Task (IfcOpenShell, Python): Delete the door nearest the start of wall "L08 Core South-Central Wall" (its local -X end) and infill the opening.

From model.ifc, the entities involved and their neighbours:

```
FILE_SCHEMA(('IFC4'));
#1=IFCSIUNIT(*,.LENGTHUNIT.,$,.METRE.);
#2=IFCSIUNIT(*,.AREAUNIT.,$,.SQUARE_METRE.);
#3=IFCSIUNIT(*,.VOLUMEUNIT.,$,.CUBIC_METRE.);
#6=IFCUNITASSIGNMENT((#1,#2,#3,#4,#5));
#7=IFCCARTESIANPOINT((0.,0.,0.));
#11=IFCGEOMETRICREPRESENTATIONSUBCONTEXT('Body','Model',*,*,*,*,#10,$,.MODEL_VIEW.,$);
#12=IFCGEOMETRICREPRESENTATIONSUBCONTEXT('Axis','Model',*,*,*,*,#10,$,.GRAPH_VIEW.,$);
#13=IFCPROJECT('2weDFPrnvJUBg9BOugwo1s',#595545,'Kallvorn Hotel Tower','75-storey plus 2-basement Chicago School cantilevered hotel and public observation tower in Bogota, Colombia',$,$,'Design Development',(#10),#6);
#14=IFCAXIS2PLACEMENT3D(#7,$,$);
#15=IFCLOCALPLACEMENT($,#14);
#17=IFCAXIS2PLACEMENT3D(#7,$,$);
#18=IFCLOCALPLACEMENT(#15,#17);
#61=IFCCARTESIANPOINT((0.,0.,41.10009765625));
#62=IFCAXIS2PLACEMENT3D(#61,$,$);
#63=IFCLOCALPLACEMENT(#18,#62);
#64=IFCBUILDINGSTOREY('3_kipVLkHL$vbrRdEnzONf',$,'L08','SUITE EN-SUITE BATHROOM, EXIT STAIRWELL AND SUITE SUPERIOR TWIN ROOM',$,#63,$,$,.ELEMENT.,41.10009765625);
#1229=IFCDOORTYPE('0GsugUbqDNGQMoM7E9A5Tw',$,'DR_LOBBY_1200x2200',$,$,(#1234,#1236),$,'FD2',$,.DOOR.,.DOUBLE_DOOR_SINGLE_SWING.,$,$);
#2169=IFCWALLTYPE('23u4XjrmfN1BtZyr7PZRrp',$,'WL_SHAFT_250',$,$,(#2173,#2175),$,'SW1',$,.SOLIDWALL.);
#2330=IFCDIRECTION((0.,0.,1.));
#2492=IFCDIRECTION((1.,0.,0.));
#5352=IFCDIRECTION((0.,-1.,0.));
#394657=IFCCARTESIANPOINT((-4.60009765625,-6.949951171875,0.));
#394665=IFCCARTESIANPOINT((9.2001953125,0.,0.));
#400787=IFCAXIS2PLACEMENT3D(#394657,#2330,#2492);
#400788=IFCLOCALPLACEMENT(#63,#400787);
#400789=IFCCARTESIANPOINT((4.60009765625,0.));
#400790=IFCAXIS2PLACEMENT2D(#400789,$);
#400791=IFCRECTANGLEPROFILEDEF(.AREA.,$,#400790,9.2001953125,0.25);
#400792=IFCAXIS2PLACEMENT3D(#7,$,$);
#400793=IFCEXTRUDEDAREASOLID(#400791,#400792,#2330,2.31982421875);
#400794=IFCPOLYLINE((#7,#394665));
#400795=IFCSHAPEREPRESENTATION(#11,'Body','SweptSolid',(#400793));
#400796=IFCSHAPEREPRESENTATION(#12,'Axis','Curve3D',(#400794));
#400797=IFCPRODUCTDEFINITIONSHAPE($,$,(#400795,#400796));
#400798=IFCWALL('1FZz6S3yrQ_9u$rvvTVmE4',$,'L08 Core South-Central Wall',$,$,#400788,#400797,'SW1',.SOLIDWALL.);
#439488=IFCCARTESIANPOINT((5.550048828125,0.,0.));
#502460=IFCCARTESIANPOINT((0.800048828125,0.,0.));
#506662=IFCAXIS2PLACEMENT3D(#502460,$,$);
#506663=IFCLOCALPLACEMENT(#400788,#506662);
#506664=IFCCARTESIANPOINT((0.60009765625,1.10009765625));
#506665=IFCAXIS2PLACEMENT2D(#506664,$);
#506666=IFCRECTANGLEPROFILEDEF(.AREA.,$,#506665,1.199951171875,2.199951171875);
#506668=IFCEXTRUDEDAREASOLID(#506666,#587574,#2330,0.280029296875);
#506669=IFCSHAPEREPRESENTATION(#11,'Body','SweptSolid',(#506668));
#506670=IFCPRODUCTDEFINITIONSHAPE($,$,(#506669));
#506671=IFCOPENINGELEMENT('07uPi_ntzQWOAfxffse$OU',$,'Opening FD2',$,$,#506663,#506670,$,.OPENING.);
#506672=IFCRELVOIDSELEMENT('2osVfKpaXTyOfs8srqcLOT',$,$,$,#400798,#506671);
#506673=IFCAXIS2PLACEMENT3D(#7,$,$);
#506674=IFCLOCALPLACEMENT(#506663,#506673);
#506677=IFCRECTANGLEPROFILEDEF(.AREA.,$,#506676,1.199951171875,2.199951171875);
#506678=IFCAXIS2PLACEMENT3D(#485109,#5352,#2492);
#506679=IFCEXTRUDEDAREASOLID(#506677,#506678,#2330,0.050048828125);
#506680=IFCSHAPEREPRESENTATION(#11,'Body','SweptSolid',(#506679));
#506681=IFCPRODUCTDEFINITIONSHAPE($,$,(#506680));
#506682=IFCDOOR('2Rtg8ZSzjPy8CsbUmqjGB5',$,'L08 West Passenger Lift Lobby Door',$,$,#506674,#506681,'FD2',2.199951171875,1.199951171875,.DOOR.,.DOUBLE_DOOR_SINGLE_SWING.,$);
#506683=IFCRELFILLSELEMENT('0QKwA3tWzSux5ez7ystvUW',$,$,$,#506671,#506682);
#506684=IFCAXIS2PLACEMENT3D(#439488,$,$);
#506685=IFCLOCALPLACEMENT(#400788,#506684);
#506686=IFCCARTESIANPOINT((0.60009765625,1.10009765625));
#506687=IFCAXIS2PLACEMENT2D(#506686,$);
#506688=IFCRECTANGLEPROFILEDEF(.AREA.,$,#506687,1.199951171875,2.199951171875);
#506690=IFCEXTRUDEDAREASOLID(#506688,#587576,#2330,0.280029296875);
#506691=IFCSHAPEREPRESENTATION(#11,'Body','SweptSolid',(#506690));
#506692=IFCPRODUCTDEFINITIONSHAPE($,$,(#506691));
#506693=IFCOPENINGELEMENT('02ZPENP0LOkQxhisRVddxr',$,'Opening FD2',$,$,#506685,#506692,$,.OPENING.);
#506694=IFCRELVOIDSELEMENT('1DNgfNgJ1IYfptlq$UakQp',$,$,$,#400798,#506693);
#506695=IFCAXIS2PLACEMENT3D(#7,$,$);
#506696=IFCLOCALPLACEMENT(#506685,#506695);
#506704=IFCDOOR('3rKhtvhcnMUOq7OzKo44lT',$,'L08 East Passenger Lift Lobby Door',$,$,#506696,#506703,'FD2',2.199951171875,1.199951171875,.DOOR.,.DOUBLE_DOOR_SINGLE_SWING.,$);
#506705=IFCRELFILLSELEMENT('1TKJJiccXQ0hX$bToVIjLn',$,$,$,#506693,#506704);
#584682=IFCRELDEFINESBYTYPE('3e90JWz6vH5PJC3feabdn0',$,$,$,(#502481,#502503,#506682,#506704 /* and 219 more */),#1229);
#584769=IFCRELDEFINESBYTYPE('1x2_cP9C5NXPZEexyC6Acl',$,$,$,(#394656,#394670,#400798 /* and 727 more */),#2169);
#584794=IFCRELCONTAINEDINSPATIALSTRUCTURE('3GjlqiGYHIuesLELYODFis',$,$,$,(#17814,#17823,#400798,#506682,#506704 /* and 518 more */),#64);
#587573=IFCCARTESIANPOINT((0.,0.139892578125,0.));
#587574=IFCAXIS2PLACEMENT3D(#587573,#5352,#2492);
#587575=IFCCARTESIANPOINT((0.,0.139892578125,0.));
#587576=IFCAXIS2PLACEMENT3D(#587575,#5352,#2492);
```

```python
import ifcopenshell
import ifcopenshell.api.feature
import ifcopenshell.api.root
import ifcopenshell.geom
import ifcopenshell.util.shape

model = ifcopenshell.open("model.ifc")
settings = ifcopenshell.geom.settings()


def volume(element):
    """Net volume in cubic metres, openings subtracted."""
    shape = ifcopenshell.geom.create_shape(settings, element)
    return ifcopenshell.util.shape.get_volume(shape.geometry)


door = model.by_guid("2Rtg8ZSzjPy8CsbUmqjGB5")
opening = door.FillsVoids[0].RelatingOpeningElement
wall = opening.VoidsElements[0].RelatingBuildingElement
before = volume(wall)

ifcopenshell.api.root.remove_product(model, product=door)
ifcopenshell.api.feature.remove_feature(model, feature=opening)

after = volume(wall)

print(f"wall volume {before:.3f} -> {after:.3f} m3")

model.write("model_edited.ifc")
```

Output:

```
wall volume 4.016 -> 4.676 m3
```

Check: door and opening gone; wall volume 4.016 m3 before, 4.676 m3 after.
